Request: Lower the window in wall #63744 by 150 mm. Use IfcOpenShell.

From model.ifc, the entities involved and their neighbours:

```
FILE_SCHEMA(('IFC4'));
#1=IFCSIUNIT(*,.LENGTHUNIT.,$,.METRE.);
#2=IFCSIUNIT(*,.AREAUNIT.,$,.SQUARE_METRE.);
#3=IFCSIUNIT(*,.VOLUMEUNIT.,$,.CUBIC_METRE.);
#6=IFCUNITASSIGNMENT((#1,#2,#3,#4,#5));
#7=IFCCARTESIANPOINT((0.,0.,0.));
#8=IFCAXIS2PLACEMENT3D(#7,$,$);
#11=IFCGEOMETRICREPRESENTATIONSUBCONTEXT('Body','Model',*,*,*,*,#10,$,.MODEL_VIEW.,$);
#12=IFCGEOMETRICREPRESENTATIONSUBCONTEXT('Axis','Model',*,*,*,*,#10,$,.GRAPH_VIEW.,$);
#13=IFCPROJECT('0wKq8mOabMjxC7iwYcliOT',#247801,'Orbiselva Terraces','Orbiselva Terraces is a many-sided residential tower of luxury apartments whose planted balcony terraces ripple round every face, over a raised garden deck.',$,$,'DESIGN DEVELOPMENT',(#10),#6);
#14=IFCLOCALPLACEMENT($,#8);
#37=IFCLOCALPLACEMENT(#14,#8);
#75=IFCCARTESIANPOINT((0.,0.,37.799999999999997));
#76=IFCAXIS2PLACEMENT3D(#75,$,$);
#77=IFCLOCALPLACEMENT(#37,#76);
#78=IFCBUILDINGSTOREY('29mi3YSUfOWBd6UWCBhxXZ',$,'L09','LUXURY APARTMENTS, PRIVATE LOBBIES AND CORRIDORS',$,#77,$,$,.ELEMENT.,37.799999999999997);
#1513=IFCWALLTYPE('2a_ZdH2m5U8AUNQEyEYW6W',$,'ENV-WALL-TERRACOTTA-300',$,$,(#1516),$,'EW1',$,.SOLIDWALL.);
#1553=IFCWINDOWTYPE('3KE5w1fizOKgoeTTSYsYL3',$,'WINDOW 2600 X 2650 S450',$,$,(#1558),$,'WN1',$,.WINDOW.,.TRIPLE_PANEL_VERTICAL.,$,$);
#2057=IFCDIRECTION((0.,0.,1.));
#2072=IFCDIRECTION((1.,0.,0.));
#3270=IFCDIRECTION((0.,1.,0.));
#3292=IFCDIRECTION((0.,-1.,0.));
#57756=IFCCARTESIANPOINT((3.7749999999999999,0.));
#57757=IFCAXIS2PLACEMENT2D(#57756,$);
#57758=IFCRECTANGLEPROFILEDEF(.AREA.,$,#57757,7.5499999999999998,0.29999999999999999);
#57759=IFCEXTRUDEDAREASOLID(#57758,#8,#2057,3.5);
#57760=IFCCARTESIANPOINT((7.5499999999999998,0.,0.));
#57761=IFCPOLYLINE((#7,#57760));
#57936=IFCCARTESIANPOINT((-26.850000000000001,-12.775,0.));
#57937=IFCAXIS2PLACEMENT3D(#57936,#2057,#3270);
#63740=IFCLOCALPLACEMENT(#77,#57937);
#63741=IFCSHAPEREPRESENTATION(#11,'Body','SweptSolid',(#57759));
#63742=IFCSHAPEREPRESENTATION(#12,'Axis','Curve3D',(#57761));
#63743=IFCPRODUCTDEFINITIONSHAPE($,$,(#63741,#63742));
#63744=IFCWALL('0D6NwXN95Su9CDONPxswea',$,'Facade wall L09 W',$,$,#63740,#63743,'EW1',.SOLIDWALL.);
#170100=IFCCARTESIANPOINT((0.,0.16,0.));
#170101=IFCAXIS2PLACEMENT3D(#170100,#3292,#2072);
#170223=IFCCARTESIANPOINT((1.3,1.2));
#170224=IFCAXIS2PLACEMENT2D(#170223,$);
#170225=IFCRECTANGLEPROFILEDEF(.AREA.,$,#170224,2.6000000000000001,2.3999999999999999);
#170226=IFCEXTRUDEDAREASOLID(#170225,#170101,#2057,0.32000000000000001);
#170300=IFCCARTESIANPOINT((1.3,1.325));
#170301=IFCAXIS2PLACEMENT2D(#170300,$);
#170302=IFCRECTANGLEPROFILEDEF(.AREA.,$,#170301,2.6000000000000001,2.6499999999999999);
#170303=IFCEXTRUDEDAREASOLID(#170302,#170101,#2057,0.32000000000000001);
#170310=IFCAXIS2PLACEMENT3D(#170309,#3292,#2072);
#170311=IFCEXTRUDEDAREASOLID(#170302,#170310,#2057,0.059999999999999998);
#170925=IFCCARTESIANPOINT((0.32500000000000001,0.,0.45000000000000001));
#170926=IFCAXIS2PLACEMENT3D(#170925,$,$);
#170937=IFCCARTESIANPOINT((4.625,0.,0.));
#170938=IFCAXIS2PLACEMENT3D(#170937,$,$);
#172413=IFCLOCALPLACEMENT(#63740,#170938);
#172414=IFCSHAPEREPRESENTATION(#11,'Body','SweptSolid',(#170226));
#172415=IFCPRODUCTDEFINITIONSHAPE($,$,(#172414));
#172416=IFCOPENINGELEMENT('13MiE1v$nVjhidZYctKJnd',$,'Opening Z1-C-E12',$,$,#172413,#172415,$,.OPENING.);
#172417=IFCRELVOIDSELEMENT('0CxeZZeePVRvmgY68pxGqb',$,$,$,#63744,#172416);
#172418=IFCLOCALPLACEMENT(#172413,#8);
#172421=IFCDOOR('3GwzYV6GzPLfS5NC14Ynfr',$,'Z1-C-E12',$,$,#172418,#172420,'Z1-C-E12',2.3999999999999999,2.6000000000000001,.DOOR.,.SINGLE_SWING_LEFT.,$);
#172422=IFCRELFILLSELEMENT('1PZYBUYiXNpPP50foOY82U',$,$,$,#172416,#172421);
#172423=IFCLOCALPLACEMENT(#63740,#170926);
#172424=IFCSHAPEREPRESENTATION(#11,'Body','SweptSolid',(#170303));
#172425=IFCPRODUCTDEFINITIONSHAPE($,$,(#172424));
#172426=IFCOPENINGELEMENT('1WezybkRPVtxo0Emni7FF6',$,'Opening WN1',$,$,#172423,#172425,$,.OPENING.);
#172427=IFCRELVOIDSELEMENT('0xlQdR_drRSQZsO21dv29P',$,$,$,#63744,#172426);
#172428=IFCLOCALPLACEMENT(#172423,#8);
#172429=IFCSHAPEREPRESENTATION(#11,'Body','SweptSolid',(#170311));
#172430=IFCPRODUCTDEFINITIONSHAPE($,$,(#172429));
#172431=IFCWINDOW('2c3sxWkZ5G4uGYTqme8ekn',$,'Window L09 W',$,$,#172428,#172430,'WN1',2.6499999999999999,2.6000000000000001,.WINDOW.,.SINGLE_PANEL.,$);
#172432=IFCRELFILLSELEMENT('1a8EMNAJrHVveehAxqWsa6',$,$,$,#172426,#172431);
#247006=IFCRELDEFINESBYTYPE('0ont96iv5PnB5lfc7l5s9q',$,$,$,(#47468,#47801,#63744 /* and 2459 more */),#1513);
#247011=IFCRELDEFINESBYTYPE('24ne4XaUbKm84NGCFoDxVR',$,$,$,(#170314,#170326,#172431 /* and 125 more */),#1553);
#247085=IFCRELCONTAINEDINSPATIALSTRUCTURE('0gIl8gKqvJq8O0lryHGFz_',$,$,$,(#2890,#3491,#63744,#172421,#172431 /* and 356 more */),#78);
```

```python
import numpy as np
import ifcopenshell
import ifcopenshell.api.geometry
import ifcopenshell.util.placement
import ifcopenshell.util.unit

model = ifcopenshell.open("model.ifc")
unit_scale = ifcopenshell.util.unit.calculate_unit_scale(model)

window = model.by_guid("2c3sxWkZ5G4uGYTqme8ekn")
opening = window.FillsVoids[0].RelatingOpeningElement
dz = -0.15

shift = np.array([0.0, 0.0, dz])
# The window is placed relative to its opening, so it follows when the opening moves.
matrix = ifcopenshell.util.placement.get_local_placement(opening.ObjectPlacement)
matrix[:3, 3] += shift
ifcopenshell.api.geometry.edit_object_placement(
    model, product=opening, matrix=matrix, is_si=False, should_transform_children=True
)

print(f"moved by {dz * unit_scale:+.3f} m")

model.write("model_rev.ifc")
```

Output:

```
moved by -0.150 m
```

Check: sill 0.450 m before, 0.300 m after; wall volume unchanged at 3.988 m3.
